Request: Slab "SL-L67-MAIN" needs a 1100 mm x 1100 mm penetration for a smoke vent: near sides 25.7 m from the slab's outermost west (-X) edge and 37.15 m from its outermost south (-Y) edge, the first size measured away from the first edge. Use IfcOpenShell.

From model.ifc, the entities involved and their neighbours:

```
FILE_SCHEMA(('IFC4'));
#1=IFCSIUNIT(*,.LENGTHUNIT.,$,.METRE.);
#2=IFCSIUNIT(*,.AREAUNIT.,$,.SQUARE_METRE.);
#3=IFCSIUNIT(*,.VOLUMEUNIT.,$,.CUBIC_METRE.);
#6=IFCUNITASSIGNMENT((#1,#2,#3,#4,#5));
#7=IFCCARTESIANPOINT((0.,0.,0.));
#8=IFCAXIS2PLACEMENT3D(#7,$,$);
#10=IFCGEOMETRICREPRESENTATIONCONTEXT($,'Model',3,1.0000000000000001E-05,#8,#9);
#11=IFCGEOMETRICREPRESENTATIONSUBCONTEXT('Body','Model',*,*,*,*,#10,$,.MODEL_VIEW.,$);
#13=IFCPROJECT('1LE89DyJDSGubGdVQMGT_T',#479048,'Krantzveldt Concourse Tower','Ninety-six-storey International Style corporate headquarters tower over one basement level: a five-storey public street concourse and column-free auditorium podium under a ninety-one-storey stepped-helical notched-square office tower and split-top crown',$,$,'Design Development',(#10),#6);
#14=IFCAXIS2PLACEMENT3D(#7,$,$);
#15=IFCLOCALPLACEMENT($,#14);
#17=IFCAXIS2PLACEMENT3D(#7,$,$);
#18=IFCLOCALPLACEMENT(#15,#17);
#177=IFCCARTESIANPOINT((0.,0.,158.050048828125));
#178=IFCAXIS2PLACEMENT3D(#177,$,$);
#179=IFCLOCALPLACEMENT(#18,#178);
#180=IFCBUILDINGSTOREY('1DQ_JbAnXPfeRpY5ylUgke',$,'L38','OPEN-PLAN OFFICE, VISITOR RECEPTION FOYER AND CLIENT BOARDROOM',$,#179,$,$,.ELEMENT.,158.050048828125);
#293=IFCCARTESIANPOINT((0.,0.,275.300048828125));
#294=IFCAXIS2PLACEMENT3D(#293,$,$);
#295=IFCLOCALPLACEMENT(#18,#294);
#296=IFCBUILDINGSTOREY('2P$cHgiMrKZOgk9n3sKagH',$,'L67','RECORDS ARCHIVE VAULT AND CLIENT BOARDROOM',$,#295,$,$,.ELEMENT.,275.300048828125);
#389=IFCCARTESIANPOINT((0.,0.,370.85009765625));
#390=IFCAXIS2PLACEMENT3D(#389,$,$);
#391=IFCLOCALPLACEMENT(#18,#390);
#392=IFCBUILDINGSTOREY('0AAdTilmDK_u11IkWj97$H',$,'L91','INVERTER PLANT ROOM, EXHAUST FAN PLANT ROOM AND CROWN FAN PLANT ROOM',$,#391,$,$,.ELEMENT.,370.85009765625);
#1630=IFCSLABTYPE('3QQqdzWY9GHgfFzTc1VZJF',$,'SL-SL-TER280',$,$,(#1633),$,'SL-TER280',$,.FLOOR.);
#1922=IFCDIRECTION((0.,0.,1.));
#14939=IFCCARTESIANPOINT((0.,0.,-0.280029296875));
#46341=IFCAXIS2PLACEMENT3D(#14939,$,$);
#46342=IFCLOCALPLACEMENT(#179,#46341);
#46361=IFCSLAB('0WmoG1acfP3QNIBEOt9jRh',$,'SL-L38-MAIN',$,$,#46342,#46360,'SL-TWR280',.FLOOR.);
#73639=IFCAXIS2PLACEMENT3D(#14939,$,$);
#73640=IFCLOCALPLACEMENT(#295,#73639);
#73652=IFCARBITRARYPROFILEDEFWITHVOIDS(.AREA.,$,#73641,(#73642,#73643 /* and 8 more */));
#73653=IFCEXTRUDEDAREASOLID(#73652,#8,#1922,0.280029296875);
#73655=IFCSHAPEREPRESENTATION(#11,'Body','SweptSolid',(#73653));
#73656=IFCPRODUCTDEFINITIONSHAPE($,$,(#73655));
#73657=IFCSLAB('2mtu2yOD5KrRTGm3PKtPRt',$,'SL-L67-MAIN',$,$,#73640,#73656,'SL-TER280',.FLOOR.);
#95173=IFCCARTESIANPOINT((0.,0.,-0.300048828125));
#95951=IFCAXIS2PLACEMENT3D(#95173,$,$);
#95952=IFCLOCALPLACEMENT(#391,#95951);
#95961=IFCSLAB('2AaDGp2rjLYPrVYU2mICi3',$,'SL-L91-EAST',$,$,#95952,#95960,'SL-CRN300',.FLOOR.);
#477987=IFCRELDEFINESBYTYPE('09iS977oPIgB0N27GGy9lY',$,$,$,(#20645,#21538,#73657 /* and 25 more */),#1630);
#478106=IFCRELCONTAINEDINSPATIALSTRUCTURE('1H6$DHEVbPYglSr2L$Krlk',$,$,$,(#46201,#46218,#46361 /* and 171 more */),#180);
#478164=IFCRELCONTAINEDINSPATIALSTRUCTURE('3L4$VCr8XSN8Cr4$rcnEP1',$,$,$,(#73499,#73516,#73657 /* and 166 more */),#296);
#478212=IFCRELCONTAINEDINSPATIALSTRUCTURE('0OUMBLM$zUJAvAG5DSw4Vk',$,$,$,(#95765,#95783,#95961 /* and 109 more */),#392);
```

```python
import numpy as np
import ifcopenshell
import ifcopenshell.api.feature
import ifcopenshell.api.geometry
import ifcopenshell.api.root
import ifcopenshell.geom
import ifcopenshell.util.placement
import ifcopenshell.util.representation
import ifcopenshell.util.shape
import ifcopenshell.util.unit

model = ifcopenshell.open("model.ifc")
unit_scale = ifcopenshell.util.unit.calculate_unit_scale(model)
settings = ifcopenshell.geom.settings()


def volume(element):
    """Net volume in cubic metres, openings subtracted."""
    shape = ifcopenshell.geom.create_shape(settings, element)
    return ifcopenshell.util.shape.get_volume(shape.geometry)


slab = model.by_guid("2mtu2yOD5KrRTGm3PKtPRt")
before = volume(slab)

# Extent in the slab's own axes, in metres. The edges named are its -X and -Y sides.
slab_shape = ifcopenshell.geom.create_shape(settings, slab)
vertices = ifcopenshell.util.shape.get_vertices(slab_shape.geometry)
x_min, y_min, bottom = vertices.min(axis=0)
top = vertices[:, 2].max()

opening = ifcopenshell.api.root.create_entity(model, ifc_class="IfcOpeningElement", name="Smoke vent opening", predefined_type="OPENING")
context = ifcopenshell.util.representation.get_context(model, "Model", "Body", "MODEL_VIEW")
width, depth = 1.1, 1.1
outline = [(0.0, 0.0), (width, 0.0), (width, depth), (0.0, depth), (0.0, 0.0)]
# Overshoot both faces by 50 mm so the cut is clean.
shape = ifcopenshell.api.geometry.add_slab_representation(
    model, context=context, depth=top - bottom + 0.1, polyline=outline
)
ifcopenshell.api.geometry.assign_representation(model, product=opening, representation=shape)

matrix = ifcopenshell.util.placement.get_local_placement(slab.ObjectPlacement)
matrix[:, 3] = matrix @ np.append(np.array([x_min + 25.7, y_min + 37.15, bottom - 0.05]) / unit_scale, 1.0)
ifcopenshell.api.geometry.edit_object_placement(model, product=opening, matrix=matrix, is_si=False)
ifcopenshell.api.feature.add_feature(model, feature=opening, element=slab)

after = volume(slab)

print(f"slab volume {before:.3f} -> {after:.3f} m3")

model.write("model-out.ifc")
```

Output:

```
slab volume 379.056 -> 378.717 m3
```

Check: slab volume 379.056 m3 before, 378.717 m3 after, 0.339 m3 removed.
